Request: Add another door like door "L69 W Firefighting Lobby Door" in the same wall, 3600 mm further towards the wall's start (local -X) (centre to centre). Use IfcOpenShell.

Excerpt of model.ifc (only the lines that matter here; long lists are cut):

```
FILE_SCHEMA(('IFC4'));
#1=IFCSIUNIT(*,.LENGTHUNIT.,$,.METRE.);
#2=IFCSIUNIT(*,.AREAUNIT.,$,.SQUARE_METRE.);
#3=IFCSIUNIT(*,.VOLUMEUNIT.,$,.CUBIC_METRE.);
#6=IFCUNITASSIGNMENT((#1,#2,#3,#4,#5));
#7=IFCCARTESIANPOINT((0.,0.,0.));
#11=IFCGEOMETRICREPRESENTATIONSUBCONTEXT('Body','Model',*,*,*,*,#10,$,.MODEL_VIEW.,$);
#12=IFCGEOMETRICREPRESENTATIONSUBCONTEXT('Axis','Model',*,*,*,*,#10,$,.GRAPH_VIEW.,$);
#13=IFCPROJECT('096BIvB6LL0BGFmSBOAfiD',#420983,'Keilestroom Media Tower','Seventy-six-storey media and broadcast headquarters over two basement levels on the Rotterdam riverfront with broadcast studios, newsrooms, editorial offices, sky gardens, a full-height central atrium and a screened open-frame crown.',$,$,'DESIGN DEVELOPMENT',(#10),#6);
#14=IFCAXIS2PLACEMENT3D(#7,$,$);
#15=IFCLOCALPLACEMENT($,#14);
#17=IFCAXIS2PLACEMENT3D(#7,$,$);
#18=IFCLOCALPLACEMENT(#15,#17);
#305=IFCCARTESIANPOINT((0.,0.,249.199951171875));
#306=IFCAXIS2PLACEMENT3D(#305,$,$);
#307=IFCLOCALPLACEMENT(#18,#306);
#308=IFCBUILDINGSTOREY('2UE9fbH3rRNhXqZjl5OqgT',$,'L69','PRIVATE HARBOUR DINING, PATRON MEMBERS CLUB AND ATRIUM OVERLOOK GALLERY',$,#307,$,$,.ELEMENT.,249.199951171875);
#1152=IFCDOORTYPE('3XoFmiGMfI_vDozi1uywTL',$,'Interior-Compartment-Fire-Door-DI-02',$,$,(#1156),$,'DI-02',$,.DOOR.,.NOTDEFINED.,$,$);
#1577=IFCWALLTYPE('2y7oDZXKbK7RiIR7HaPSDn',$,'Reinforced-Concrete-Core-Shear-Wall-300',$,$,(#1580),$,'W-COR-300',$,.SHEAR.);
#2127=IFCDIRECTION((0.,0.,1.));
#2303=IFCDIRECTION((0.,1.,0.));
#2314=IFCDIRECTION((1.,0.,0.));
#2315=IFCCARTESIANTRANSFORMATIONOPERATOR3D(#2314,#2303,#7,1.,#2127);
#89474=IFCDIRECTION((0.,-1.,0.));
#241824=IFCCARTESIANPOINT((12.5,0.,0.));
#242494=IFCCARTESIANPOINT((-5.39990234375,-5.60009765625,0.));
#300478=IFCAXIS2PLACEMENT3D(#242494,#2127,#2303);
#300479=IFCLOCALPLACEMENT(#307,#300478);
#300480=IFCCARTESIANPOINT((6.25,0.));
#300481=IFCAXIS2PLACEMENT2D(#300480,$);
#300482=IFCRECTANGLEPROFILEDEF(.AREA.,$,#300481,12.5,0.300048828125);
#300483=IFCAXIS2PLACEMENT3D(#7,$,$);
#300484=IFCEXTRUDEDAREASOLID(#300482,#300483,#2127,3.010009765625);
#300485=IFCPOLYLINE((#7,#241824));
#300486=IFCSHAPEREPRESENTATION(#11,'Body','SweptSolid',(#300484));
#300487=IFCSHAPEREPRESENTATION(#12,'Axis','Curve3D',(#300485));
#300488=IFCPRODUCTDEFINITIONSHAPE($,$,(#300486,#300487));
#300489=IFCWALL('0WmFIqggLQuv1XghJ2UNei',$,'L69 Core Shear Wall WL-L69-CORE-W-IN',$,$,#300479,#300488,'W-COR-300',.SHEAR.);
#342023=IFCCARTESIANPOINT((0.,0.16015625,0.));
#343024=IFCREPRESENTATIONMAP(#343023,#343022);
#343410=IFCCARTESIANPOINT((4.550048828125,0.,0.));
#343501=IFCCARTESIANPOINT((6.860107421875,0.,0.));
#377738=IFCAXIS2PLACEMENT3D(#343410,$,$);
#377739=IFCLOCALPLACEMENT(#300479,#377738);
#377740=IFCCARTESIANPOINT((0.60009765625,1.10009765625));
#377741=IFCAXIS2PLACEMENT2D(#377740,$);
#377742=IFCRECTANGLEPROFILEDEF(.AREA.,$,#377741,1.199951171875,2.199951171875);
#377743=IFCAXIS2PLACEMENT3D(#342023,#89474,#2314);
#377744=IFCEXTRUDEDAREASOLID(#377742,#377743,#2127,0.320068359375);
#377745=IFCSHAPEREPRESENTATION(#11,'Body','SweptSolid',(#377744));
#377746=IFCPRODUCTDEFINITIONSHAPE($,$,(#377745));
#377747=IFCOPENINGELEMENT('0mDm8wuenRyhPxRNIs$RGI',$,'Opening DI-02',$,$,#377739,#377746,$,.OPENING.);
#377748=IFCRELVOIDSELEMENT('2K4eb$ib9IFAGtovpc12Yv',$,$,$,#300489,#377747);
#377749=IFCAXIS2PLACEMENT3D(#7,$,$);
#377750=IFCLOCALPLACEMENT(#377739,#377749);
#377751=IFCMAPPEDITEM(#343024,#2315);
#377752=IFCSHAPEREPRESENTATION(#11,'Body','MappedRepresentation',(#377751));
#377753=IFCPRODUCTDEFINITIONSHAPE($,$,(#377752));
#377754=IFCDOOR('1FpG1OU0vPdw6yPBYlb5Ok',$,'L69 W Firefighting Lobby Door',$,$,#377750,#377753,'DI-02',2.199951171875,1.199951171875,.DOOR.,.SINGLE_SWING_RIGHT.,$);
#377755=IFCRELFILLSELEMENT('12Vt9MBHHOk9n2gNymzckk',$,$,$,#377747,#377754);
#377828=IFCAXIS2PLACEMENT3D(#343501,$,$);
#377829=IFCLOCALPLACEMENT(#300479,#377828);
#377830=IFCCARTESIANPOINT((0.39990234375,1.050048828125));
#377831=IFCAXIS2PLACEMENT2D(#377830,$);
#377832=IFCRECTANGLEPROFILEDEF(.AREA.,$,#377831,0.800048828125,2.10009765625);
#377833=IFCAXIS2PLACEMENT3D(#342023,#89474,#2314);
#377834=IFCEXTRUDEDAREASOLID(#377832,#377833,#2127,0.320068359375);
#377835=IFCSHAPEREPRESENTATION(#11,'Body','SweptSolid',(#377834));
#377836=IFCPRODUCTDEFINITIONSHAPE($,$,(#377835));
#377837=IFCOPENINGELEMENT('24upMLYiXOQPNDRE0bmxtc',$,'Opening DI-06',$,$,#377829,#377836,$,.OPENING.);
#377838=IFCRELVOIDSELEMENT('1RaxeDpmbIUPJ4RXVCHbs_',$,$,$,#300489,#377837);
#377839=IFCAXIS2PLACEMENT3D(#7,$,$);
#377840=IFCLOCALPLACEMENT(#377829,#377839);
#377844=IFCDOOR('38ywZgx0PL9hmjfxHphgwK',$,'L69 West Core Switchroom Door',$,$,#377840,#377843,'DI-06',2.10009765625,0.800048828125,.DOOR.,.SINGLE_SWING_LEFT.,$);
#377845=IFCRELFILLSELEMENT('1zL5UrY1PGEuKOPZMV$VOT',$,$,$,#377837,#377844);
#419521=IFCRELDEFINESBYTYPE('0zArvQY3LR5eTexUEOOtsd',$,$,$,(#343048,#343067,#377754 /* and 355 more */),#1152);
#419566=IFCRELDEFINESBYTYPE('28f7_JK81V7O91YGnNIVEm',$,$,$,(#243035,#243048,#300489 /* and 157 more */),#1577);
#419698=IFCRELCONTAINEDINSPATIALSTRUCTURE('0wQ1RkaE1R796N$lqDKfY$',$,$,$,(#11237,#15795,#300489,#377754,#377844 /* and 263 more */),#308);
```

```python
import ifcopenshell
import ifcopenshell.api.feature
import ifcopenshell.api.geometry
import ifcopenshell.api.root
import ifcopenshell.geom
import ifcopenshell.util.element
import ifcopenshell.util.placement
import ifcopenshell.util.shape
import ifcopenshell.util.unit

model = ifcopenshell.open("model.ifc")
unit_scale = ifcopenshell.util.unit.calculate_unit_scale(model)
settings = ifcopenshell.geom.settings()


def volume(element):
    """Net volume in cubic metres, openings subtracted."""
    shape = ifcopenshell.geom.create_shape(settings, element)
    return ifcopenshell.util.shape.get_volume(shape.geometry)


door = model.by_id(377754)
opening = door.FillsVoids[0].RelatingOpeningElement
wall = opening.VoidsElements[0].RelatingBuildingElement
before = volume(wall)
shift = ifcopenshell.util.placement.get_local_placement(wall.ObjectPlacement)[:3, 0] * -3.6 / unit_scale

# copy_class copies the void relationship, type, container and properties, but no geometry.
new_opening = ifcopenshell.api.root.copy_class(model, product=opening)
new_opening.Representation = ifcopenshell.util.element.copy_deep(
    model, opening.Representation, exclude=["IfcGeometricRepresentationContext", "IfcRepresentationMap"]
)
new_door = ifcopenshell.api.root.copy_class(model, product=door)
new_door.Representation = ifcopenshell.util.element.copy_deep(
    model, door.Representation, exclude=["IfcGeometricRepresentationContext", "IfcRepresentationMap"]
)
new_door.Tag = None
ifcopenshell.api.feature.add_filling(model, opening=new_opening, element=new_door)

for old, new in ((opening, new_opening), (door, new_door)):
    matrix = ifcopenshell.util.placement.get_local_placement(old.ObjectPlacement)
    matrix[:3, 3] += shift
    ifcopenshell.api.geometry.edit_object_placement(model, product=new, matrix=matrix, is_si=False)

after = volume(wall)

print(f"wall volume {before:.3f} -> {after:.3f} m3")

model.write("model_rev.ifc")
```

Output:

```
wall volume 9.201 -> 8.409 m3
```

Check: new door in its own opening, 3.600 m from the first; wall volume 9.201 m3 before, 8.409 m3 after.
